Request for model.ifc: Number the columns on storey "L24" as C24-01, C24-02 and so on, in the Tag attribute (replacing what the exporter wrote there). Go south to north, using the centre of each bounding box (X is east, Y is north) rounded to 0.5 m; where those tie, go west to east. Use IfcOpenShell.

First a look at what the model holds.

```python
import ifcopenshell
import ifcopenshell.util.element
import ifcopenshell.util.placement

model = ifcopenshell.open("model.ifc")
print(model.schema)
storey = next(s for s in model.by_type("IfcBuildingStorey") if s.Name == "L24")
columns = [e for e in ifcopenshell.util.element.get_decomposition(storey) if e.is_a("IfcColumn")]
for e in sorted(columns, key=lambda e: e.id()):
    origin = ifcopenshell.util.placement.get_local_placement(e.ObjectPlacement)[:3, 3]
    print(e.id(), e.Tag, e.Name, origin.round(2) + 0.0, sep=" | ")
```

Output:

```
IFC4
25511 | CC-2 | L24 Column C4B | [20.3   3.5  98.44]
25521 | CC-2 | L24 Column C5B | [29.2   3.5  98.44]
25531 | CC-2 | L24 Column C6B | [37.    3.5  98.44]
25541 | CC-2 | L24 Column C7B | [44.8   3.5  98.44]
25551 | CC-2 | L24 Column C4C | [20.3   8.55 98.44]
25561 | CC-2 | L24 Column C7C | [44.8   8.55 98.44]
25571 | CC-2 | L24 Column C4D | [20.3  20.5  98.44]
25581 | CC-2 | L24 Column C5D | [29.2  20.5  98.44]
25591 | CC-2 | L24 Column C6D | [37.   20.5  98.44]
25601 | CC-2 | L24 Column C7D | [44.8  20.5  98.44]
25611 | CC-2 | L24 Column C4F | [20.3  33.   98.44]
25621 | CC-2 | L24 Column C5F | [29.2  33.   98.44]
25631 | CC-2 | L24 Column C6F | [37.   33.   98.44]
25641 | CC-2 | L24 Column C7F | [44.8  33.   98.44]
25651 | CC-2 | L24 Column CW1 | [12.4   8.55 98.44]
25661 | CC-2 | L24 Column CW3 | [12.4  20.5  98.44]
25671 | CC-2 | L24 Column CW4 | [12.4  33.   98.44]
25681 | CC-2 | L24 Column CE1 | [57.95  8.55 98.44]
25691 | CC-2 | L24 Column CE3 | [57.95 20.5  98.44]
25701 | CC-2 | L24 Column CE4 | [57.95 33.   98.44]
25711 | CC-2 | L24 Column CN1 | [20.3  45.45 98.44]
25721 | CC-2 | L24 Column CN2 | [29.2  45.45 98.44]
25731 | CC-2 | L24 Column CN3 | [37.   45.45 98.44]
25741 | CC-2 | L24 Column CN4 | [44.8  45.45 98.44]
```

```python
import ifcopenshell
import ifcopenshell.geom
import ifcopenshell.util.element
import ifcopenshell.util.shape

model = ifcopenshell.open("model.ifc")
settings = ifcopenshell.geom.settings()
settings.set("use-world-coords", True)


def centre(element):
    shape = ifcopenshell.geom.create_shape(settings, element)
    return ifcopenshell.util.shape.get_bbox_centroid(shape.geometry)


storey = next(s for s in model.by_type("IfcBuildingStorey") if s.Name == "L24")
columns = [e for e in ifcopenshell.util.element.get_decomposition(storey) if e.is_a("IfcColumn")]

# Insertion points can sit at a corner or the storey origin, so sort by the geometry (in metres).
centres = {e: centre(e) for e in columns}
columns.sort(key=lambda e: (round(centres[e][1] / 0.5), centres[e][0]))

for i, e in enumerate(columns, start=1):
    number = f"C24-{i:02d}"
    e.Tag = number
    print(e.id(), number)

model.write("model_updated.ifc")
```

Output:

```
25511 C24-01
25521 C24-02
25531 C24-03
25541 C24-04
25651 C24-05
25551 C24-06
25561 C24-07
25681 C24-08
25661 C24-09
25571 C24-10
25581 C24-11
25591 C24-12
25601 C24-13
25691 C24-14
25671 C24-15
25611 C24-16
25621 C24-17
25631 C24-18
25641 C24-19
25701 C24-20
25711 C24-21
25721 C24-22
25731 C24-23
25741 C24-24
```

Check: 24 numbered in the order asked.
